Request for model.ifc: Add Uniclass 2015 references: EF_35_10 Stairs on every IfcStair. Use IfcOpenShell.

First a look at what the model holds.

```python
import ifcopenshell

model = ifcopenshell.open("model.ifc")
print(model.schema)
print("classifications:", [c.Name for c in model.by_type("IfcClassification")])
for ifc_class in ("IfcDoor", "IfcRoof", "IfcStair", "IfcWall", "IfcWindow"):
    print(ifc_class, len(model.by_type(ifc_class)))
```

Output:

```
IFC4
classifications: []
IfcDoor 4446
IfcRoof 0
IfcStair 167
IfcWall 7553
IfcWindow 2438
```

```python
import ifcopenshell
import ifcopenshell.api.classification

model = ifcopenshell.open("model.ifc")

system = ifcopenshell.api.classification.add_classification(model, classification="Uniclass 2015")

codes = {
    "IfcStair": ("EF_35_10", "Stairs"),
}
for ifc_class, (code, name) in codes.items():
    products = model.by_type(ifc_class)
    ifcopenshell.api.classification.add_reference(
        model, products=products, classification=system, identification=code, name=name
    )
    print(code, len(products))

model.write("model_updated.ifc")
```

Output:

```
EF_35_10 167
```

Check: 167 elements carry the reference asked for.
